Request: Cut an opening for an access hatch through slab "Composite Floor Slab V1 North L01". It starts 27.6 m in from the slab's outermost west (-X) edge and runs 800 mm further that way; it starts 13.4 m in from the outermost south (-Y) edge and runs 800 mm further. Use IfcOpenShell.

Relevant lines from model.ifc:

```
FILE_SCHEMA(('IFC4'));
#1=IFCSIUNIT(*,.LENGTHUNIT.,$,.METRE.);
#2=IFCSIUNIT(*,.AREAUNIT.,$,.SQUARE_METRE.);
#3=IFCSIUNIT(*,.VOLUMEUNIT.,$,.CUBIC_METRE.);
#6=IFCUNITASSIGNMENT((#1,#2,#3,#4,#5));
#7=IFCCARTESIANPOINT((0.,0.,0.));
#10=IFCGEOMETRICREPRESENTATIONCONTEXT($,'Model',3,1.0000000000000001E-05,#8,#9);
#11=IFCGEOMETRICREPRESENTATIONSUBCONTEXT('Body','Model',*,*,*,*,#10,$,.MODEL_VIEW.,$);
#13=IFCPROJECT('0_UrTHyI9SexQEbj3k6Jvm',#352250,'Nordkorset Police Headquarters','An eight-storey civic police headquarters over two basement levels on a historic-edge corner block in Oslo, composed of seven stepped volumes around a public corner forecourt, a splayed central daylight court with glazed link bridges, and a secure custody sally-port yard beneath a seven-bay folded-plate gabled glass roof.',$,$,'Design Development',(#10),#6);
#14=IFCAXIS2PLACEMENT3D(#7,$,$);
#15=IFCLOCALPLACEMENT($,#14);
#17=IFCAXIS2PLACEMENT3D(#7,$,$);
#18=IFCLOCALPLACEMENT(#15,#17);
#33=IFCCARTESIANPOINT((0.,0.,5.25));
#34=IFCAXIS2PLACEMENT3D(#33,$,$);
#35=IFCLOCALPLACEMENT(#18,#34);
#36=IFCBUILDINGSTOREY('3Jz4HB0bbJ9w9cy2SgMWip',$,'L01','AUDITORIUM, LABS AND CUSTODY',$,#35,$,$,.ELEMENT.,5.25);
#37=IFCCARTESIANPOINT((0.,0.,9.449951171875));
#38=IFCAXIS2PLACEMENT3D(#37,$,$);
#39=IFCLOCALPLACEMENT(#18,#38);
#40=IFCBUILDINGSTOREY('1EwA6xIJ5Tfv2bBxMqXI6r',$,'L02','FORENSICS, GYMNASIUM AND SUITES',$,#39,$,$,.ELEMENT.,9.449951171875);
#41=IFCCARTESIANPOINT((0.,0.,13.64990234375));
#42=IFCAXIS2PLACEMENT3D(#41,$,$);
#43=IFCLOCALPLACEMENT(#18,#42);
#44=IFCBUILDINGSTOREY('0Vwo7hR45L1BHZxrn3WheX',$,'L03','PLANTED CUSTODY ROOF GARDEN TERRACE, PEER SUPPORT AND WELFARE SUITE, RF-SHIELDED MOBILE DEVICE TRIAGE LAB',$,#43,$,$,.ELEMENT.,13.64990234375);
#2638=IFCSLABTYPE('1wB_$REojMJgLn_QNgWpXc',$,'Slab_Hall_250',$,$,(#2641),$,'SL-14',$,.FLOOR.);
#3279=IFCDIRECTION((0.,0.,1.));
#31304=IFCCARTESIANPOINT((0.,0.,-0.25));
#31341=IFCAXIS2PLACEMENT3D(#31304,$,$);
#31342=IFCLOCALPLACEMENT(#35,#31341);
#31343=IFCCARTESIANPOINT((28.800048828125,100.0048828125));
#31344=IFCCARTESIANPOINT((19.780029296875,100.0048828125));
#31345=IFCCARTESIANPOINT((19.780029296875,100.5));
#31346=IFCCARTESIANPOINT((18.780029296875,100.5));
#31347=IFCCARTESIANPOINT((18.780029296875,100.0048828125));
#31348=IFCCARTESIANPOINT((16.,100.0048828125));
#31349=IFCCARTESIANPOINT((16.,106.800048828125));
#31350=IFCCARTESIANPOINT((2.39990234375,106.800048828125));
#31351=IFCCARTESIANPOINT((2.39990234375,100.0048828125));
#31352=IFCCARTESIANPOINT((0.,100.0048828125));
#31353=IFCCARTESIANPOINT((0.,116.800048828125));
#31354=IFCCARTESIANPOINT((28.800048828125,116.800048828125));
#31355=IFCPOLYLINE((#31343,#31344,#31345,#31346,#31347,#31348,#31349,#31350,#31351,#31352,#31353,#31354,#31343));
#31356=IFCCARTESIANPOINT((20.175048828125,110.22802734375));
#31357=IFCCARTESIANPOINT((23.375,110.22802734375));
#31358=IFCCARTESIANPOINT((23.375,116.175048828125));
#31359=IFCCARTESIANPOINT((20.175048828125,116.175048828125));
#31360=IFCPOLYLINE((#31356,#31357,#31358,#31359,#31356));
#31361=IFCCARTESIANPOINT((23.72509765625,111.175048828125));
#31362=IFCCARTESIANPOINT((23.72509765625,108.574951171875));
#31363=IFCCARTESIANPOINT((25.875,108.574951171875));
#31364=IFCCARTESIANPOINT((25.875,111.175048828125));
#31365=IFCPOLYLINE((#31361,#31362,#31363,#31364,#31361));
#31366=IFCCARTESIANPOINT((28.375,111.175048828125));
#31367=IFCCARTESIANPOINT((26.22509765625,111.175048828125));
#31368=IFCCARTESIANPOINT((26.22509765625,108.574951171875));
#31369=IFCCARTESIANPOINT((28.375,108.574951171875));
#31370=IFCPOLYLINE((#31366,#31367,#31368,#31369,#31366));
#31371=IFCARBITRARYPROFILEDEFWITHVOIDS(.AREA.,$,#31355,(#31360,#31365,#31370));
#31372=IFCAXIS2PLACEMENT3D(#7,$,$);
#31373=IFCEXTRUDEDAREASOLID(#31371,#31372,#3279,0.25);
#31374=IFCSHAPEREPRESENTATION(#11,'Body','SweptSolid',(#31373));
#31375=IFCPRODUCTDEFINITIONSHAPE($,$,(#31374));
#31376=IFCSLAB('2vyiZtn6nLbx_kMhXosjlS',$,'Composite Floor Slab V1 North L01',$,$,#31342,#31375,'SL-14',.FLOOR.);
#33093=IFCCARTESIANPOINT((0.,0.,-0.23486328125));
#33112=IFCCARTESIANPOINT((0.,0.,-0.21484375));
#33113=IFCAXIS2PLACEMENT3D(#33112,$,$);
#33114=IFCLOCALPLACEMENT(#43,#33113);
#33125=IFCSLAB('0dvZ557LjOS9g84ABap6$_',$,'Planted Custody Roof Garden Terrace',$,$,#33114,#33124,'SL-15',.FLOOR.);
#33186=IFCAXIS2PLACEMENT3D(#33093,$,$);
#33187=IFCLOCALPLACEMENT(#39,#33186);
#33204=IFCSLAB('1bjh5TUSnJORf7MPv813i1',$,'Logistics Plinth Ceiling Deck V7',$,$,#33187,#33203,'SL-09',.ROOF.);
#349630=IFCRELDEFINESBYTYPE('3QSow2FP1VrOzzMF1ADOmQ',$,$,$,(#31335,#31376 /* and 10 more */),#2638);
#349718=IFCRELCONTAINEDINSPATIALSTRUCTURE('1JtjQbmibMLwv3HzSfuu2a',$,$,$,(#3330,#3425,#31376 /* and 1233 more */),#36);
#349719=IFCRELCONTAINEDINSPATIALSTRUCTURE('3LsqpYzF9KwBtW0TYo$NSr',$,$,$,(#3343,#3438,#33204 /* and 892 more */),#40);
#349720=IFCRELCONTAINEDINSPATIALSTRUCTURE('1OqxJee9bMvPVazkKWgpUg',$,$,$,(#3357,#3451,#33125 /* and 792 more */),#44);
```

```python
import numpy as np
import ifcopenshell
import ifcopenshell.api.feature
import ifcopenshell.api.geometry
import ifcopenshell.api.root
import ifcopenshell.geom
import ifcopenshell.util.placement
import ifcopenshell.util.representation
import ifcopenshell.util.shape
import ifcopenshell.util.unit

model = ifcopenshell.open("model.ifc")
unit_scale = ifcopenshell.util.unit.calculate_unit_scale(model)
settings = ifcopenshell.geom.settings()


def volume(element):
    """Net volume in cubic metres, openings subtracted."""
    shape = ifcopenshell.geom.create_shape(settings, element)
    return ifcopenshell.util.shape.get_volume(shape.geometry)


slab = model.by_guid("2vyiZtn6nLbx_kMhXosjlS")
before = volume(slab)

# Extent in the slab's own axes, in metres. The edges named are its -X and -Y sides.
slab_shape = ifcopenshell.geom.create_shape(settings, slab)
vertices = ifcopenshell.util.shape.get_vertices(slab_shape.geometry)
x_min, y_min, bottom = vertices.min(axis=0)
top = vertices[:, 2].max()

opening = ifcopenshell.api.root.create_entity(model, ifc_class="IfcOpeningElement", name="Access hatch opening", predefined_type="OPENING")
context = ifcopenshell.util.representation.get_context(model, "Model", "Body", "MODEL_VIEW")
width, depth = 0.8, 0.8
outline = [(0.0, 0.0), (width, 0.0), (width, depth), (0.0, depth), (0.0, 0.0)]
# Overshoot both faces by 50 mm so the cut is clean.
shape = ifcopenshell.api.geometry.add_slab_representation(
    model, context=context, depth=top - bottom + 0.1, polyline=outline
)
ifcopenshell.api.geometry.assign_representation(model, product=opening, representation=shape)

matrix = ifcopenshell.util.placement.get_local_placement(slab.ObjectPlacement)
matrix[:, 3] = matrix @ np.append(np.array([x_min + 27.6, y_min + 13.4, bottom - 0.05]) / unit_scale, 1.0)
ifcopenshell.api.geometry.edit_object_placement(model, product=opening, matrix=matrix, is_si=False)
ifcopenshell.api.feature.add_feature(model, feature=opening, element=slab)

after = volume(slab)

print(f"slab volume {before:.3f} -> {after:.3f} m3")

model.write("model_updated.ifc")
```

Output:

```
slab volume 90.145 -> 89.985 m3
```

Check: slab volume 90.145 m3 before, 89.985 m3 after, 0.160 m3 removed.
